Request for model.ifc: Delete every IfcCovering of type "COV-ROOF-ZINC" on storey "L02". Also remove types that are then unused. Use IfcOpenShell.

First a look at what the model holds.

```python
import ifcopenshell
import ifcopenshell.util.element

model = ifcopenshell.open("model.ifc")
print(model.schema)
storey = next(s for s in model.by_type("IfcBuildingStorey") if s.Name == "L02")
coverings = [e for e in ifcopenshell.util.element.get_decomposition(storey) if e.is_a("IfcCovering")]
seen = {}
for e in coverings:
    element_type = ifcopenshell.util.element.get_type(e)
    name = element_type.Name if element_type not in (None, e) else None
    seen[name] = seen.get(name, 0) + 1
for name, count in sorted(seen.items(), key=str):
    print(count, "x", name)
```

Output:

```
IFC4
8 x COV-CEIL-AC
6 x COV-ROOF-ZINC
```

```python
import ifcopenshell
import ifcopenshell.api.root
import ifcopenshell.util.element

model = ifcopenshell.open("model.ifc")

storey = next(s for s in model.by_type("IfcBuildingStorey") if s.Name == "L02")
coverings = [e for e in ifcopenshell.util.element.get_decomposition(storey) if e.is_a("IfcCovering")]
targets = [e for e in coverings if (t := ifcopenshell.util.element.get_type(e)) not in (None, e) and t.Name == "COV-ROOF-ZINC"]
types = {ifcopenshell.util.element.get_type(e) for e in targets} - {None, *targets}

for e in targets:
    ifcopenshell.api.root.remove_product(model, product=e)
print(len(targets), "removed")

unused = [t for t in types if not ifcopenshell.util.element.get_types(t)]
for t in unused:
    ifcopenshell.api.root.remove_product(model, product=t)
print(len(unused), "unused types removed")

model.write("model-out.ifc")
```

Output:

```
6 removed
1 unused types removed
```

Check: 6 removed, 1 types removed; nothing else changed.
